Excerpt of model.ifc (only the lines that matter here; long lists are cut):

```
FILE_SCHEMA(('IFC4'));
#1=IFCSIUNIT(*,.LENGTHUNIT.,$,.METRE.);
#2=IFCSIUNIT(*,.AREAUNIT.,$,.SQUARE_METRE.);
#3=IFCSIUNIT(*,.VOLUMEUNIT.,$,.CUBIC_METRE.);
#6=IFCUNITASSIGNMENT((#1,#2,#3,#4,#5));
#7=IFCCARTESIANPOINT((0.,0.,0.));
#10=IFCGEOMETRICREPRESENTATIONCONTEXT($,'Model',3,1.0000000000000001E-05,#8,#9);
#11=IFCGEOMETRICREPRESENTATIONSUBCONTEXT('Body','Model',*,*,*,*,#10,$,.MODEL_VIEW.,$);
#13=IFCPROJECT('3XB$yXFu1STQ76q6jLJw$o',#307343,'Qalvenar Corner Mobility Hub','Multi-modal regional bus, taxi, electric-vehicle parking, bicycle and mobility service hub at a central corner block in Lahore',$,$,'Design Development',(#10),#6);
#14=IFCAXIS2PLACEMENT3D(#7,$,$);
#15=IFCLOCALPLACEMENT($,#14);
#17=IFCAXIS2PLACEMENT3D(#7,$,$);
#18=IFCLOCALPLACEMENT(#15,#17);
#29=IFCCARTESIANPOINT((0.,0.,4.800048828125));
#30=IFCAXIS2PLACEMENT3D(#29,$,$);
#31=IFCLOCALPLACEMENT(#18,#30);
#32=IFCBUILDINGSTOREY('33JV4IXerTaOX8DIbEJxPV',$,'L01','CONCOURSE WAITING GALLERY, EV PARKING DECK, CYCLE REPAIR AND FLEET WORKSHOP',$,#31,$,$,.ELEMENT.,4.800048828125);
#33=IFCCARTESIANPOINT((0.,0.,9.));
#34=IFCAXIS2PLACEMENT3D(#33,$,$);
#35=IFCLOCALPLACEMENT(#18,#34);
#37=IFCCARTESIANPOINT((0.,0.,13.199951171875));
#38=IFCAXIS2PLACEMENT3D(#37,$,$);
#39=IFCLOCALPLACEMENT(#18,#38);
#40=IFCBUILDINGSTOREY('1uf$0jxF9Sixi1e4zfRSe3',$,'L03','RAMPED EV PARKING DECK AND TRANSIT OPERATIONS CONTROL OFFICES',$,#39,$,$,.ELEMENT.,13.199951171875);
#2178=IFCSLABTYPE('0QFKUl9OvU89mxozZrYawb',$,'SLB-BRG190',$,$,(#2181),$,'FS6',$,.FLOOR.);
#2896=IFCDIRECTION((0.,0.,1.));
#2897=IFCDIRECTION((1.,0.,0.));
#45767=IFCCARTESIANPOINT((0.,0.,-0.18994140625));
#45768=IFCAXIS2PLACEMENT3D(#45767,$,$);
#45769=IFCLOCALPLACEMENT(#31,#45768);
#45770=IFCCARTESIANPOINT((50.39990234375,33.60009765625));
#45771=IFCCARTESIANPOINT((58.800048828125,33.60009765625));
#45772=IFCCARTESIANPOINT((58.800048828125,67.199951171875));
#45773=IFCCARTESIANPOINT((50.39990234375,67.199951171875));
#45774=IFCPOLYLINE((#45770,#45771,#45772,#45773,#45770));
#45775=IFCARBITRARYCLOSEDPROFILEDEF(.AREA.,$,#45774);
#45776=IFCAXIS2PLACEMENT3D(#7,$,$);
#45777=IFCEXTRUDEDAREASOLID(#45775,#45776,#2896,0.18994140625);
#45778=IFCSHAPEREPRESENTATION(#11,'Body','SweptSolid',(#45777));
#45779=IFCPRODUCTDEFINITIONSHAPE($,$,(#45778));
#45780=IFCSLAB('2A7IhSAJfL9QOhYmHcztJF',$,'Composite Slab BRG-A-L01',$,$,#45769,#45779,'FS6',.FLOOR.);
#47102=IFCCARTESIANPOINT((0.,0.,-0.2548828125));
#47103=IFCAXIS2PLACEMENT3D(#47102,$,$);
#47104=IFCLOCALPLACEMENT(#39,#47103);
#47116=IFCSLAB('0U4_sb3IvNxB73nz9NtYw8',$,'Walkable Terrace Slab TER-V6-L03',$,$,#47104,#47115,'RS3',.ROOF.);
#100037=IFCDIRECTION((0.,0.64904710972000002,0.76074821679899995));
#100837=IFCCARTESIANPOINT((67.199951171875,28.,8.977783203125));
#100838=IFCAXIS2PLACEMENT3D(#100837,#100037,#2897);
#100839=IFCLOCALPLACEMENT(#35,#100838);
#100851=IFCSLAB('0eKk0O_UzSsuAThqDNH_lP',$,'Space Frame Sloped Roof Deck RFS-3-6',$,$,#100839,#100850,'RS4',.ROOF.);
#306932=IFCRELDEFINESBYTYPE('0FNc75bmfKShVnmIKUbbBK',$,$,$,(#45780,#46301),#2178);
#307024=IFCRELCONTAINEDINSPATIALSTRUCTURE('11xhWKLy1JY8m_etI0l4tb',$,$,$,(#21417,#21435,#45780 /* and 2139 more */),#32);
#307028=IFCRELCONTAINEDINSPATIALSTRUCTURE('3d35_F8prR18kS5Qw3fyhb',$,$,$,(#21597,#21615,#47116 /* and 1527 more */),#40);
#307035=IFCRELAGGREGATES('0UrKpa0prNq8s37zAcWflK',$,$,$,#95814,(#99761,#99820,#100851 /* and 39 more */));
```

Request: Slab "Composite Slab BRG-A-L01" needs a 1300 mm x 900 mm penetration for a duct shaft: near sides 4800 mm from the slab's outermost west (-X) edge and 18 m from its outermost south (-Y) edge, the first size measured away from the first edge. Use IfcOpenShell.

```python
import numpy as np
import ifcopenshell
import ifcopenshell.api.feature
import ifcopenshell.api.geometry
import ifcopenshell.api.root
import ifcopenshell.geom
import ifcopenshell.util.placement
import ifcopenshell.util.representation
import ifcopenshell.util.shape
import ifcopenshell.util.unit

model = ifcopenshell.open("model.ifc")
unit_scale = ifcopenshell.util.unit.calculate_unit_scale(model)
settings = ifcopenshell.geom.settings()


def volume(element):
    """Net volume in cubic metres, openings subtracted."""
    shape = ifcopenshell.geom.create_shape(settings, element)
    return ifcopenshell.util.shape.get_volume(shape.geometry)


slab = model.by_id(45780)
before = volume(slab)

# Extent in the slab's own axes, in metres. The edges named are its -X and -Y sides.
slab_shape = ifcopenshell.geom.create_shape(settings, slab)
vertices = ifcopenshell.util.shape.get_vertices(slab_shape.geometry)
x_min, y_min, bottom = vertices.min(axis=0)
top = vertices[:, 2].max()

opening = ifcopenshell.api.root.create_entity(model, ifc_class="IfcOpeningElement", name="Duct shaft opening", predefined_type="OPENING")
context = ifcopenshell.util.representation.get_context(model, "Model", "Body", "MODEL_VIEW")
width, depth = 1.3, 0.9
outline = [(0.0, 0.0), (width, 0.0), (width, depth), (0.0, depth), (0.0, 0.0)]
# Overshoot both faces by 50 mm so the cut is clean.
shape = ifcopenshell.api.geometry.add_slab_representation(
    model, context=context, depth=top - bottom + 0.1, polyline=outline
)
ifcopenshell.api.geometry.assign_representation(model, product=opening, representation=shape)

matrix = ifcopenshell.util.placement.get_local_placement(slab.ObjectPlacement)
matrix[:, 3] = matrix @ np.append(np.array([x_min + 4.8, y_min + 18, bottom - 0.05]) / unit_scale, 1.0)
ifcopenshell.api.geometry.edit_object_placement(model, product=opening, matrix=matrix, is_si=False)
ifcopenshell.api.feature.add_feature(model, feature=opening, element=slab)

after = volume(slab)

print(f"slab volume {before:.3f} -> {after:.3f} m3")

model.write("model_v2.ifc")
```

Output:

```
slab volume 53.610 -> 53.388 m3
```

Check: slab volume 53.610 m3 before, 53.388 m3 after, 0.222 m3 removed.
